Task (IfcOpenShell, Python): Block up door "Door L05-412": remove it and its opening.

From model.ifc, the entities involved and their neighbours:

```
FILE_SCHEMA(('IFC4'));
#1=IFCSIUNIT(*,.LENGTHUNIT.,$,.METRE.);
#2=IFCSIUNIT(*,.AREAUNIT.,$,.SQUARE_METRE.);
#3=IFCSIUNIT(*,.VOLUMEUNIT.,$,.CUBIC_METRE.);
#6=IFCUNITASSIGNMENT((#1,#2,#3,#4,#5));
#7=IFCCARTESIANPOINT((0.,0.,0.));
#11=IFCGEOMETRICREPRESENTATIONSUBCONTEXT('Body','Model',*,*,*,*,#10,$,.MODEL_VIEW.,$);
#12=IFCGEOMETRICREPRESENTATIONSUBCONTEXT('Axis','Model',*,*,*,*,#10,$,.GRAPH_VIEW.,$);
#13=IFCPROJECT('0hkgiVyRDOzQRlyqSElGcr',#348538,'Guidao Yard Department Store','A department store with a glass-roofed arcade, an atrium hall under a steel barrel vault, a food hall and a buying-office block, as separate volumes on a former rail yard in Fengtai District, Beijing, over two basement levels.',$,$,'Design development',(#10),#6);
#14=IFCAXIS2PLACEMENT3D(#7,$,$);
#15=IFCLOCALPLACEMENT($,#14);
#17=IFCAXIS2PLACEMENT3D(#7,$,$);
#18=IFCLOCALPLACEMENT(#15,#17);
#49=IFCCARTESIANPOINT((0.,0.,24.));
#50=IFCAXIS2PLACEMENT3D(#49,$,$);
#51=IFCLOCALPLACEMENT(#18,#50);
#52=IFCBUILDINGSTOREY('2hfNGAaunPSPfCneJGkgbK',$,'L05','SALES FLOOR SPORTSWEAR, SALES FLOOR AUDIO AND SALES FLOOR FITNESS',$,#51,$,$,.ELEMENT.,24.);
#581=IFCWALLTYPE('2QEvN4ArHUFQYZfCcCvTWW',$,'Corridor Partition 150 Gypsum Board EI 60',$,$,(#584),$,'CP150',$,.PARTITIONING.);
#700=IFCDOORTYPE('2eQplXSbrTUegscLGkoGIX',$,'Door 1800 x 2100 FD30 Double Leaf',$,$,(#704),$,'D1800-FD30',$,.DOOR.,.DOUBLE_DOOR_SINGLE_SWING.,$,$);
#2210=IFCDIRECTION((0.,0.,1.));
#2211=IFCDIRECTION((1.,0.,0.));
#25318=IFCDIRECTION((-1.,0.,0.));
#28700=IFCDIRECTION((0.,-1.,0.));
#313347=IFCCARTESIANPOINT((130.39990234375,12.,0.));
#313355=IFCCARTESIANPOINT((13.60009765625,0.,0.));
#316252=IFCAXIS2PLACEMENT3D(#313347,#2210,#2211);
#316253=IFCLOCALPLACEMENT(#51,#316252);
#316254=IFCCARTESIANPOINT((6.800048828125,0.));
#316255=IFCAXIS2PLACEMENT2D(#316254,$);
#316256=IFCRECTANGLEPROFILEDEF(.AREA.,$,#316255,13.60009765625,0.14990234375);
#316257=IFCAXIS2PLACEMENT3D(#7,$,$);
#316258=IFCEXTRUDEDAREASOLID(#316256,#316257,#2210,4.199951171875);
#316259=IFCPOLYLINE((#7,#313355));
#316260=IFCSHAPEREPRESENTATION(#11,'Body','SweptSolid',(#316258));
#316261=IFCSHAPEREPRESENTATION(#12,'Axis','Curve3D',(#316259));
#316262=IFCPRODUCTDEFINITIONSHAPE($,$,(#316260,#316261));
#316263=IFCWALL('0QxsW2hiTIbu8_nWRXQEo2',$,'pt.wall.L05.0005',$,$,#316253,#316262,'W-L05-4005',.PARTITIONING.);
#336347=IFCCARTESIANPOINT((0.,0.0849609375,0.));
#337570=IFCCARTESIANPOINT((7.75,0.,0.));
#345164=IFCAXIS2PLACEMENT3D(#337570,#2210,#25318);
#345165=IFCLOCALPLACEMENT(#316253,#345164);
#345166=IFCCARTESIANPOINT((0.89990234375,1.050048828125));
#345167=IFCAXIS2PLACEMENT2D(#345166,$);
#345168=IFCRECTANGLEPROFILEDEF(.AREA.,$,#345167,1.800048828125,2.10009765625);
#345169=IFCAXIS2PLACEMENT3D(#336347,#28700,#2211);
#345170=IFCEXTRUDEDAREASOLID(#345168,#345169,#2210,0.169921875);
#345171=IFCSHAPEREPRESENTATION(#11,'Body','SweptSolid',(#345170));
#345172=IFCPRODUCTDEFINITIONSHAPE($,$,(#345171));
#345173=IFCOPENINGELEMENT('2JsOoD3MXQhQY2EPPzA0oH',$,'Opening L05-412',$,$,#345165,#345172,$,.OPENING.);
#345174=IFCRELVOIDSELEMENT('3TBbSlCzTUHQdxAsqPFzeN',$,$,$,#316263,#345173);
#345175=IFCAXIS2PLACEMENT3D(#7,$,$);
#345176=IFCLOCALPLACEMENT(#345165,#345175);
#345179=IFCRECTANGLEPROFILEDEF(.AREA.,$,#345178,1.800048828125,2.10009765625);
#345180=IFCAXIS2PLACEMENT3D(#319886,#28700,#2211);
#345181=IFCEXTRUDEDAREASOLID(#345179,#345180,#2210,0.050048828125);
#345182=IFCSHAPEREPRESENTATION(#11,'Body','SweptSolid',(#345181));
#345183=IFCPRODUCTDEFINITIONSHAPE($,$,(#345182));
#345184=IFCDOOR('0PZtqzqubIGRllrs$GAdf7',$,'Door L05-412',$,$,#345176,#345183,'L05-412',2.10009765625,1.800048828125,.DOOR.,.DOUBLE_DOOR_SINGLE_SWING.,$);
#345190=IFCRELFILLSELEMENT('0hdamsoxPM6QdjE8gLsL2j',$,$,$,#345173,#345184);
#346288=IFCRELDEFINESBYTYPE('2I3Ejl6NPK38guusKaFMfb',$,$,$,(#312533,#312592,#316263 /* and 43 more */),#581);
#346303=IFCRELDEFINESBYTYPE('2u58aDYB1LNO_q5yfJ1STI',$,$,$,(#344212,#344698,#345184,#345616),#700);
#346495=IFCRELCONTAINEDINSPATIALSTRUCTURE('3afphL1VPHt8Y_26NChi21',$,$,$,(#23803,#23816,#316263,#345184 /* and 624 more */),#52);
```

```python
import ifcopenshell
import ifcopenshell.api.feature
import ifcopenshell.api.root
import ifcopenshell.geom
import ifcopenshell.util.shape

model = ifcopenshell.open("model.ifc")
settings = ifcopenshell.geom.settings()


def volume(element):
    """Net volume in cubic metres, openings subtracted."""
    shape = ifcopenshell.geom.create_shape(settings, element)
    return ifcopenshell.util.shape.get_volume(shape.geometry)


door = model.by_guid("0PZtqzqubIGRllrs$GAdf7")
opening = door.FillsVoids[0].RelatingOpeningElement
wall = opening.VoidsElements[0].RelatingBuildingElement
before = volume(wall)

ifcopenshell.api.root.remove_product(model, product=door)
ifcopenshell.api.feature.remove_feature(model, feature=opening)

after = volume(wall)

print(f"wall volume {before:.3f} -> {after:.3f} m3")

model.write("model-out.ifc")
```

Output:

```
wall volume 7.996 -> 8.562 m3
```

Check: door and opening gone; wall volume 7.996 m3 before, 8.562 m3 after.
